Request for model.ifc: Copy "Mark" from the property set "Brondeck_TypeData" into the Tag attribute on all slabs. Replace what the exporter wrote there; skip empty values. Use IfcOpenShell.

First a look at what the model holds.

```python
import ifcopenshell
import ifcopenshell.util.element

model = ifcopenshell.open("model.ifc")
print(model.schema)
slabs = model.by_type("IfcSlab")
print(len(slabs), "slabs")
for e in slabs[:8]:
    source = ifcopenshell.util.element.get_pset(e, "Brondeck_TypeData", "Mark")
    target = e.Tag
    print(e.id(), repr(source), repr(target), sep=" | ")
```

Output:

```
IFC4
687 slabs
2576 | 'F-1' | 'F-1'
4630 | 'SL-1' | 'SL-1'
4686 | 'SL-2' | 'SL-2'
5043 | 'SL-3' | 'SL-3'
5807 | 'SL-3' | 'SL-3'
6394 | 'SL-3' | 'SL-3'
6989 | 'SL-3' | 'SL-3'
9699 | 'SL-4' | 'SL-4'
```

```python
import ifcopenshell
import ifcopenshell.util.element

model = ifcopenshell.open("model.ifc")

count = 0
for e in model.by_type("IfcSlab"):
    value = ifcopenshell.util.element.get_pset(e, "Brondeck_TypeData", "Mark")
    current = e.Tag
    if not value or not value.strip() or current == value:
        continue
    e.Tag = value
    count += 1

print(count, "slabs updated")

model.write("model_edited.ifc")
```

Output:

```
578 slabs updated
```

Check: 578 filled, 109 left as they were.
